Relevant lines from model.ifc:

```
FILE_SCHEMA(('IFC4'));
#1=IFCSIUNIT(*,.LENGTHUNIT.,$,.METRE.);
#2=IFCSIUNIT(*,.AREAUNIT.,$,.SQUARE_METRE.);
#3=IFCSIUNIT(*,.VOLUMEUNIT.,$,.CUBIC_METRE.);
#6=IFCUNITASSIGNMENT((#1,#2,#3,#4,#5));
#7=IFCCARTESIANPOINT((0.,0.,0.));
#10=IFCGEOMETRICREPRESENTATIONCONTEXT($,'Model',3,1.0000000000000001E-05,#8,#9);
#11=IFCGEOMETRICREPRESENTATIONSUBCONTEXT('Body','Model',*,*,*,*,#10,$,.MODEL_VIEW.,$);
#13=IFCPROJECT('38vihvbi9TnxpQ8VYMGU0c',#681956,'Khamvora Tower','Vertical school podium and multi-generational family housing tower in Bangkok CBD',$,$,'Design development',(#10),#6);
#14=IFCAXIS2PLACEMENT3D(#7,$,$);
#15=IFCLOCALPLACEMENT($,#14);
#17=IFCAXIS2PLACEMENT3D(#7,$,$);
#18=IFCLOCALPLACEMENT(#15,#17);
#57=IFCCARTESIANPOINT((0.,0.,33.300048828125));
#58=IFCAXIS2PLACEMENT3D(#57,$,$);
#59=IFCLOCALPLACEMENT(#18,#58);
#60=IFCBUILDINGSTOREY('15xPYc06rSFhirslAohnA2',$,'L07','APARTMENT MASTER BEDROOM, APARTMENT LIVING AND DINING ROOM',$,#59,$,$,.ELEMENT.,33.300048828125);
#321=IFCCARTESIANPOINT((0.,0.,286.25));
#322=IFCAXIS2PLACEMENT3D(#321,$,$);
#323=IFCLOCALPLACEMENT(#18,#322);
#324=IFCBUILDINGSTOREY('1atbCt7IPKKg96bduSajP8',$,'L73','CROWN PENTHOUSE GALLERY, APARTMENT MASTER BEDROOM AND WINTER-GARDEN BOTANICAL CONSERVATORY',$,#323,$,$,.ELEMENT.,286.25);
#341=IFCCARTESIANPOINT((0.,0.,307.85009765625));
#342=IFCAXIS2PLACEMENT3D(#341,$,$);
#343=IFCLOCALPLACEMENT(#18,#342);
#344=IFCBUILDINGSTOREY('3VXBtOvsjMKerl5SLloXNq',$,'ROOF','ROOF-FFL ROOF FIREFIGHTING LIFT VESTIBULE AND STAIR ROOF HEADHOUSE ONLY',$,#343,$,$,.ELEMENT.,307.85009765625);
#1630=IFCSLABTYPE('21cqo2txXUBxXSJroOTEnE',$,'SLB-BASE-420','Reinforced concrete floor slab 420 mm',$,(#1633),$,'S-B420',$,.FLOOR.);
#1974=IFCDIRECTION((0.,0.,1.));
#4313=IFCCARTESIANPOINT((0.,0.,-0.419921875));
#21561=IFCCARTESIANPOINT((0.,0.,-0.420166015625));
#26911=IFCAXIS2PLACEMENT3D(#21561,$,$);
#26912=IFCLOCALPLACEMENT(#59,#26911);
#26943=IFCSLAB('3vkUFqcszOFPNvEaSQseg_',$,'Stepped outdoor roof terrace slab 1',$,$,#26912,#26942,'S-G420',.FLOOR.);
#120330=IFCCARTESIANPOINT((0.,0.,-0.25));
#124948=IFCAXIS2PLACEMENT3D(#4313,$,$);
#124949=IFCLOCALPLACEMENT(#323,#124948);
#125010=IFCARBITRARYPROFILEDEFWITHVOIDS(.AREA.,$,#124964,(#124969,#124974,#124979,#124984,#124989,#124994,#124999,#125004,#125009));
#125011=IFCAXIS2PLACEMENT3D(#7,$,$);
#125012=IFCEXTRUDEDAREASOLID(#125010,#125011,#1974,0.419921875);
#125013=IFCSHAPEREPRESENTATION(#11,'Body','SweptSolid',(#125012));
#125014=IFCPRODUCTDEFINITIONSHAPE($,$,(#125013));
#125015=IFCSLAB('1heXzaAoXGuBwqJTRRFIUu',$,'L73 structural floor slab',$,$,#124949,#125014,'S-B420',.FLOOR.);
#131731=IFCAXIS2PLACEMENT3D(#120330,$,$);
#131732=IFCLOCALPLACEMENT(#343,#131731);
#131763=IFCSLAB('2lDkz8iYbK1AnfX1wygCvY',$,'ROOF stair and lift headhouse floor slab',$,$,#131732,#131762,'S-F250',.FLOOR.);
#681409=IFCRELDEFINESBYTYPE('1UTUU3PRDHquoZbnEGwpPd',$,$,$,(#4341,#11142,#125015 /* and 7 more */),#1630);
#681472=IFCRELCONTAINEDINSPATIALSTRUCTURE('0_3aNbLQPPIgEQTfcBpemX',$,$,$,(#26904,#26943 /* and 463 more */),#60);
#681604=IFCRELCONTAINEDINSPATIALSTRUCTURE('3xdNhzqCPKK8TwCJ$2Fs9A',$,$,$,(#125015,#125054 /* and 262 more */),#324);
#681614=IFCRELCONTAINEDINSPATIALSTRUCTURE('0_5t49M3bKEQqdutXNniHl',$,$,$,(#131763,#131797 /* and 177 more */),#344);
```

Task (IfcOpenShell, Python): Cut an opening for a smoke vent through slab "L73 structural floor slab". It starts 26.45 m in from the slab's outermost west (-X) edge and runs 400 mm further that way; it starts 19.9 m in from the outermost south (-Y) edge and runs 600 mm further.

```python
import numpy as np
import ifcopenshell
import ifcopenshell.api.feature
import ifcopenshell.api.geometry
import ifcopenshell.api.root
import ifcopenshell.geom
import ifcopenshell.util.placement
import ifcopenshell.util.representation
import ifcopenshell.util.shape
import ifcopenshell.util.unit

model = ifcopenshell.open("model.ifc")
unit_scale = ifcopenshell.util.unit.calculate_unit_scale(model)
settings = ifcopenshell.geom.settings()


def volume(element):
    """Net volume in cubic metres, openings subtracted."""
    shape = ifcopenshell.geom.create_shape(settings, element)
    return ifcopenshell.util.shape.get_volume(shape.geometry)


slab = model.by_guid("1heXzaAoXGuBwqJTRRFIUu")
before = volume(slab)

# Extent in the slab's own axes, in metres. The edges named are its -X and -Y sides.
slab_shape = ifcopenshell.geom.create_shape(settings, slab)
vertices = ifcopenshell.util.shape.get_vertices(slab_shape.geometry)
x_min, y_min, bottom = vertices.min(axis=0)
top = vertices[:, 2].max()

opening = ifcopenshell.api.root.create_entity(model, ifc_class="IfcOpeningElement", name="Smoke vent opening", predefined_type="OPENING")
context = ifcopenshell.util.representation.get_context(model, "Model", "Body", "MODEL_VIEW")
width, depth = 0.4, 0.6
outline = [(0.0, 0.0), (width, 0.0), (width, depth), (0.0, depth), (0.0, 0.0)]
# Overshoot both faces by 50 mm so the cut is clean.
shape = ifcopenshell.api.geometry.add_slab_representation(
    model, context=context, depth=top - bottom + 0.1, polyline=outline
)
ifcopenshell.api.geometry.assign_representation(model, product=opening, representation=shape)

matrix = ifcopenshell.util.placement.get_local_placement(slab.ObjectPlacement)
matrix[:, 3] = matrix @ np.append(np.array([x_min + 26.45, y_min + 19.9, bottom - 0.05]) / unit_scale, 1.0)
ifcopenshell.api.geometry.edit_object_placement(model, product=opening, matrix=matrix, is_si=False)
ifcopenshell.api.feature.add_feature(model, feature=opening, element=slab)

after = volume(slab)

print(f"slab volume {before:.3f} -> {after:.3f} m3")

model.write("model-out.ifc")
```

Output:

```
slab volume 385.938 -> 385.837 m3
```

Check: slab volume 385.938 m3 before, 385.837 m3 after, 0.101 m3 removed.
